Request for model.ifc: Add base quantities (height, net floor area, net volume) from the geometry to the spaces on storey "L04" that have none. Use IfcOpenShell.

First a look at what the model holds.

```python
import ifcopenshell
import ifcopenshell.util.element
import ifcopenshell.util.unit

model = ifcopenshell.open("model.ifc")
print(model.schema)
for unit_type in ("LENGTHUNIT", "AREAUNIT", "VOLUMEUNIT"):
    print(unit_type, ifcopenshell.util.unit.calculate_unit_scale(model, unit_type))
storey = next(s for s in model.by_type("IfcBuildingStorey") if s.Name == "L04")
spaces = [e for e in ifcopenshell.util.element.get_decomposition(storey) if e.is_a("IfcSpace")]
for e in sorted(spaces, key=lambda e: e.id()):
    print(e.id(), e.is_a(), e.Name, list(ifcopenshell.util.element.get_psets(e, qtos_only=True)), sep=" | ")
```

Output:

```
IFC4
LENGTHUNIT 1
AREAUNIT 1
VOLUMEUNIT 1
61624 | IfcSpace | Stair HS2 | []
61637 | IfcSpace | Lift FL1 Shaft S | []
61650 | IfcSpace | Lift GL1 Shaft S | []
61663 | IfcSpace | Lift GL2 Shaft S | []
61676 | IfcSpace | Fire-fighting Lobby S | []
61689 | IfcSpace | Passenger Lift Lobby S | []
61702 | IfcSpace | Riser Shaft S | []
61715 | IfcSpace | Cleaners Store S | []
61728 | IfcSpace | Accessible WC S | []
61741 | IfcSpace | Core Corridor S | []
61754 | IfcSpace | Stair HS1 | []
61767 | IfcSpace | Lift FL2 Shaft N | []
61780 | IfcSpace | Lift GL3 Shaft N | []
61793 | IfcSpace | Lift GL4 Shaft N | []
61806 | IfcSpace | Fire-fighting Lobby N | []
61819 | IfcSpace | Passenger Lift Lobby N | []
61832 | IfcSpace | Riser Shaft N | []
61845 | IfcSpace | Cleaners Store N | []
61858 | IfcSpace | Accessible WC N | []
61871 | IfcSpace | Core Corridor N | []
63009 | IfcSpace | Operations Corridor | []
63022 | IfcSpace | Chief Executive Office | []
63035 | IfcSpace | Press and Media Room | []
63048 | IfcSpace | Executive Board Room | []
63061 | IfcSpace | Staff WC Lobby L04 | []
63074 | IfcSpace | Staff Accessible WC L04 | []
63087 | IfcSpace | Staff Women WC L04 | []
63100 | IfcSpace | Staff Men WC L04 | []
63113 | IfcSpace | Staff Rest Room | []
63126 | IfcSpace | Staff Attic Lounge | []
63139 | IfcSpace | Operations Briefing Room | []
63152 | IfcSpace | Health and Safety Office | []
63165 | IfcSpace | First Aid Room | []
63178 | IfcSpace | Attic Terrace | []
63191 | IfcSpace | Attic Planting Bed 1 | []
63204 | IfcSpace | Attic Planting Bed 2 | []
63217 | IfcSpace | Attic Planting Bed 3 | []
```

```python
import ifcopenshell
import ifcopenshell.api.pset
import ifcopenshell.geom
import ifcopenshell.util.element
import ifcopenshell.util.shape
import ifcopenshell.util.unit

model = ifcopenshell.open("model.ifc")
unit_scale = ifcopenshell.util.unit.calculate_unit_scale(model)
area_scale = ifcopenshell.util.unit.calculate_unit_scale(model, "AREAUNIT")
volume_scale = ifcopenshell.util.unit.calculate_unit_scale(model, "VOLUMEUNIT")
settings = ifcopenshell.geom.settings()

storey = next(s for s in model.by_type("IfcBuildingStorey") if s.Name == "L04")
spaces = [e for e in ifcopenshell.util.element.get_decomposition(storey) if e.is_a("IfcSpace")]

for e in sorted(spaces, key=lambda e: e.id()):
    if ifcopenshell.util.element.get_psets(e, qtos_only=True, should_inherit=False):
        continue
    # Geometry comes back in metres, in the element's own axes.
    shape = ifcopenshell.geom.create_shape(settings, e)
    values = {
        "Height": ifcopenshell.util.shape.get_z(shape.geometry) / unit_scale,
        "NetFloorArea": ifcopenshell.util.shape.get_footprint_area(shape.geometry) / area_scale,
        "NetVolume": ifcopenshell.util.shape.get_volume(shape.geometry) / volume_scale,
    }
    qto = ifcopenshell.api.pset.add_qto(model, product=e, name="Qto_SpaceBaseQuantities")
    ifcopenshell.api.pset.edit_qto(model, qto=qto, properties=values)
    print(e.id(), {k: round(v, 3) for k, v in values.items()})

model.write("model_updated.ifc")
```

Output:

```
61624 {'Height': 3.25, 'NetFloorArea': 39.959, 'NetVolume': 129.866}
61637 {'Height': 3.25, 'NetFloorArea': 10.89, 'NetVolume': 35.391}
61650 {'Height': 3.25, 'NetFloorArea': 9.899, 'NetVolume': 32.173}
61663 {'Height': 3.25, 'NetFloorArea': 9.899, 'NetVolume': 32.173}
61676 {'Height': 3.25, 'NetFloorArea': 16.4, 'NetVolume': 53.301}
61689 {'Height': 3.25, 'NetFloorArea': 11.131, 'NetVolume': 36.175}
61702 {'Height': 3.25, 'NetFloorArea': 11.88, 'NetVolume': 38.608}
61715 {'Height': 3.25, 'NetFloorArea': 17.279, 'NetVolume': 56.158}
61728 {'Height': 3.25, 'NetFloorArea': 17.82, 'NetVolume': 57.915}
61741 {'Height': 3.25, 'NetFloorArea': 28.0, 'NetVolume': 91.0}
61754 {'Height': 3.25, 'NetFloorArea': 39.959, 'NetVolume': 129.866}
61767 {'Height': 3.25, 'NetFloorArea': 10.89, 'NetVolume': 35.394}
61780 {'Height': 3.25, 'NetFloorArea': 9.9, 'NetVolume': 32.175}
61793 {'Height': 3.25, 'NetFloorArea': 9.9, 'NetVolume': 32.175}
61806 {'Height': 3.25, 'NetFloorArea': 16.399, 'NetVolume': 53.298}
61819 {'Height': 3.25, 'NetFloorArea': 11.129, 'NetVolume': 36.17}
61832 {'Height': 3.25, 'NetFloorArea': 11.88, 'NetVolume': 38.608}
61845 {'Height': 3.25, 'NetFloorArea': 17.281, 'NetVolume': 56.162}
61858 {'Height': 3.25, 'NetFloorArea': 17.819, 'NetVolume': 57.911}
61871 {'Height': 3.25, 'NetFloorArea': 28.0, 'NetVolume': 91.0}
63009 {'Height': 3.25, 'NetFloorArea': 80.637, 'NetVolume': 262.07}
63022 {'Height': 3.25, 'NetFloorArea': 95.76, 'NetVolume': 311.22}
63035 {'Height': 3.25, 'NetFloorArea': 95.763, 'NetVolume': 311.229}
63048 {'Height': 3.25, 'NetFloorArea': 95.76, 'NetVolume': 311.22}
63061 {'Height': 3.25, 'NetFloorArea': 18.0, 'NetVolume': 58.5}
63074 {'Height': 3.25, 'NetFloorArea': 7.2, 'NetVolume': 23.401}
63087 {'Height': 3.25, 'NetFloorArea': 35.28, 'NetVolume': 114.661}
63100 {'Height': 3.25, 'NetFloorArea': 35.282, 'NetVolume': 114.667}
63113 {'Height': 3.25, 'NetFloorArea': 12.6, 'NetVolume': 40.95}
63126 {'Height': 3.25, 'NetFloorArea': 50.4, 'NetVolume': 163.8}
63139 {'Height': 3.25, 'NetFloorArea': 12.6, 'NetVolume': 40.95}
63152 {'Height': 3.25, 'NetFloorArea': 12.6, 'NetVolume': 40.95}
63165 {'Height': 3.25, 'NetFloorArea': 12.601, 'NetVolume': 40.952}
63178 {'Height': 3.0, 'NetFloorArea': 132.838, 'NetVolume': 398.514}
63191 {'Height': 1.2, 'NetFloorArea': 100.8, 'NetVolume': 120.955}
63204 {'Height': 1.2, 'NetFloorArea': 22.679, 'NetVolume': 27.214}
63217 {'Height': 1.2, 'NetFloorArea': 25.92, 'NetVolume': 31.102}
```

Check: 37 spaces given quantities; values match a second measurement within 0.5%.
